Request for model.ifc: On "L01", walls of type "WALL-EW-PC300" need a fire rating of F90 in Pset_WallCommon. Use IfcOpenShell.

First a look at what the model holds.

```python
import ifcopenshell
import ifcopenshell.util.element

model = ifcopenshell.open("model.ifc")
print(model.schema)
storey = next(s for s in model.by_type("IfcBuildingStorey") if s.Name == "L01")
walls = [e for e in ifcopenshell.util.element.get_decomposition(storey) if e.is_a("IfcWall")]
seen = {}
for e in walls:
    element_type = ifcopenshell.util.element.get_type(e)
    key = (element_type.Name if element_type != e and element_type else None, ifcopenshell.util.element.get_pset(e, "Pset_WallCommon", "FireRating"))
    seen[key] = seen.get(key, 0) + 1
for (name, value), count in sorted(seen.items(), key=str):
    print(count, "x", name, "|", value)
```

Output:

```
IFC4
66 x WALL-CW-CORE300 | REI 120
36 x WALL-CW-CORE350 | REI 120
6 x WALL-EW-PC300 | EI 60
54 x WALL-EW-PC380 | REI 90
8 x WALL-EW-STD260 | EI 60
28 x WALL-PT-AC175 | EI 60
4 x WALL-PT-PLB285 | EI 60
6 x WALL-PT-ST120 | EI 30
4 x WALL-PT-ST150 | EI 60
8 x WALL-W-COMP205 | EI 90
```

```python
import ifcopenshell
import ifcopenshell.api.pset
import ifcopenshell.util.element

model = ifcopenshell.open("model.ifc")

storey = next(s for s in model.by_type("IfcBuildingStorey") if s.Name == "L01")
walls = [e for e in ifcopenshell.util.element.get_decomposition(storey) if e.is_a("IfcWall")]

count = 0
for e in walls:
    element_type = ifcopenshell.util.element.get_type(e)
    if element_type in (None, e) or element_type.Name != "WALL-EW-PC300":
        continue
    # add_pset returns the element's existing set when there is one.
    pset = ifcopenshell.api.pset.add_pset(model, product=e, name="Pset_WallCommon")
    ifcopenshell.api.pset.edit_pset(model, pset=pset, properties={"FireRating": "F90"})
    count += 1

print(count, "walls updated")

model.write("model-out.ifc")
```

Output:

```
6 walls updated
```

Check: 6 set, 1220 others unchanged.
